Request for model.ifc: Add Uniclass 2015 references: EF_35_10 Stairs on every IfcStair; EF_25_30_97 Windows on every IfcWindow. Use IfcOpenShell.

First a look at what the model holds.

```python
import ifcopenshell

model = ifcopenshell.open("model.ifc")
print(model.schema)
print("classifications:", [c.Name for c in model.by_type("IfcClassification")])
for ifc_class in ("IfcDoor", "IfcRoof", "IfcStair", "IfcWall", "IfcWindow"):
    print(ifc_class, len(model.by_type(ifc_class)))
```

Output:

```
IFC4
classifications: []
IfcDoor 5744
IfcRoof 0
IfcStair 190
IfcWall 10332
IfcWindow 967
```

```python
import ifcopenshell
import ifcopenshell.api.classification

model = ifcopenshell.open("model.ifc")

system = ifcopenshell.api.classification.add_classification(model, classification="Uniclass 2015")

codes = {
    "IfcStair": ("EF_35_10", "Stairs"),
    "IfcWindow": ("EF_25_30_97", "Windows"),
}
for ifc_class, (code, name) in codes.items():
    products = model.by_type(ifc_class)
    ifcopenshell.api.classification.add_reference(
        model, products=products, classification=system, identification=code, name=name
    )
    print(code, len(products))

model.write("model_rev.ifc")
```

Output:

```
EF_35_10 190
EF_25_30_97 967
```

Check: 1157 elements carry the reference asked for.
